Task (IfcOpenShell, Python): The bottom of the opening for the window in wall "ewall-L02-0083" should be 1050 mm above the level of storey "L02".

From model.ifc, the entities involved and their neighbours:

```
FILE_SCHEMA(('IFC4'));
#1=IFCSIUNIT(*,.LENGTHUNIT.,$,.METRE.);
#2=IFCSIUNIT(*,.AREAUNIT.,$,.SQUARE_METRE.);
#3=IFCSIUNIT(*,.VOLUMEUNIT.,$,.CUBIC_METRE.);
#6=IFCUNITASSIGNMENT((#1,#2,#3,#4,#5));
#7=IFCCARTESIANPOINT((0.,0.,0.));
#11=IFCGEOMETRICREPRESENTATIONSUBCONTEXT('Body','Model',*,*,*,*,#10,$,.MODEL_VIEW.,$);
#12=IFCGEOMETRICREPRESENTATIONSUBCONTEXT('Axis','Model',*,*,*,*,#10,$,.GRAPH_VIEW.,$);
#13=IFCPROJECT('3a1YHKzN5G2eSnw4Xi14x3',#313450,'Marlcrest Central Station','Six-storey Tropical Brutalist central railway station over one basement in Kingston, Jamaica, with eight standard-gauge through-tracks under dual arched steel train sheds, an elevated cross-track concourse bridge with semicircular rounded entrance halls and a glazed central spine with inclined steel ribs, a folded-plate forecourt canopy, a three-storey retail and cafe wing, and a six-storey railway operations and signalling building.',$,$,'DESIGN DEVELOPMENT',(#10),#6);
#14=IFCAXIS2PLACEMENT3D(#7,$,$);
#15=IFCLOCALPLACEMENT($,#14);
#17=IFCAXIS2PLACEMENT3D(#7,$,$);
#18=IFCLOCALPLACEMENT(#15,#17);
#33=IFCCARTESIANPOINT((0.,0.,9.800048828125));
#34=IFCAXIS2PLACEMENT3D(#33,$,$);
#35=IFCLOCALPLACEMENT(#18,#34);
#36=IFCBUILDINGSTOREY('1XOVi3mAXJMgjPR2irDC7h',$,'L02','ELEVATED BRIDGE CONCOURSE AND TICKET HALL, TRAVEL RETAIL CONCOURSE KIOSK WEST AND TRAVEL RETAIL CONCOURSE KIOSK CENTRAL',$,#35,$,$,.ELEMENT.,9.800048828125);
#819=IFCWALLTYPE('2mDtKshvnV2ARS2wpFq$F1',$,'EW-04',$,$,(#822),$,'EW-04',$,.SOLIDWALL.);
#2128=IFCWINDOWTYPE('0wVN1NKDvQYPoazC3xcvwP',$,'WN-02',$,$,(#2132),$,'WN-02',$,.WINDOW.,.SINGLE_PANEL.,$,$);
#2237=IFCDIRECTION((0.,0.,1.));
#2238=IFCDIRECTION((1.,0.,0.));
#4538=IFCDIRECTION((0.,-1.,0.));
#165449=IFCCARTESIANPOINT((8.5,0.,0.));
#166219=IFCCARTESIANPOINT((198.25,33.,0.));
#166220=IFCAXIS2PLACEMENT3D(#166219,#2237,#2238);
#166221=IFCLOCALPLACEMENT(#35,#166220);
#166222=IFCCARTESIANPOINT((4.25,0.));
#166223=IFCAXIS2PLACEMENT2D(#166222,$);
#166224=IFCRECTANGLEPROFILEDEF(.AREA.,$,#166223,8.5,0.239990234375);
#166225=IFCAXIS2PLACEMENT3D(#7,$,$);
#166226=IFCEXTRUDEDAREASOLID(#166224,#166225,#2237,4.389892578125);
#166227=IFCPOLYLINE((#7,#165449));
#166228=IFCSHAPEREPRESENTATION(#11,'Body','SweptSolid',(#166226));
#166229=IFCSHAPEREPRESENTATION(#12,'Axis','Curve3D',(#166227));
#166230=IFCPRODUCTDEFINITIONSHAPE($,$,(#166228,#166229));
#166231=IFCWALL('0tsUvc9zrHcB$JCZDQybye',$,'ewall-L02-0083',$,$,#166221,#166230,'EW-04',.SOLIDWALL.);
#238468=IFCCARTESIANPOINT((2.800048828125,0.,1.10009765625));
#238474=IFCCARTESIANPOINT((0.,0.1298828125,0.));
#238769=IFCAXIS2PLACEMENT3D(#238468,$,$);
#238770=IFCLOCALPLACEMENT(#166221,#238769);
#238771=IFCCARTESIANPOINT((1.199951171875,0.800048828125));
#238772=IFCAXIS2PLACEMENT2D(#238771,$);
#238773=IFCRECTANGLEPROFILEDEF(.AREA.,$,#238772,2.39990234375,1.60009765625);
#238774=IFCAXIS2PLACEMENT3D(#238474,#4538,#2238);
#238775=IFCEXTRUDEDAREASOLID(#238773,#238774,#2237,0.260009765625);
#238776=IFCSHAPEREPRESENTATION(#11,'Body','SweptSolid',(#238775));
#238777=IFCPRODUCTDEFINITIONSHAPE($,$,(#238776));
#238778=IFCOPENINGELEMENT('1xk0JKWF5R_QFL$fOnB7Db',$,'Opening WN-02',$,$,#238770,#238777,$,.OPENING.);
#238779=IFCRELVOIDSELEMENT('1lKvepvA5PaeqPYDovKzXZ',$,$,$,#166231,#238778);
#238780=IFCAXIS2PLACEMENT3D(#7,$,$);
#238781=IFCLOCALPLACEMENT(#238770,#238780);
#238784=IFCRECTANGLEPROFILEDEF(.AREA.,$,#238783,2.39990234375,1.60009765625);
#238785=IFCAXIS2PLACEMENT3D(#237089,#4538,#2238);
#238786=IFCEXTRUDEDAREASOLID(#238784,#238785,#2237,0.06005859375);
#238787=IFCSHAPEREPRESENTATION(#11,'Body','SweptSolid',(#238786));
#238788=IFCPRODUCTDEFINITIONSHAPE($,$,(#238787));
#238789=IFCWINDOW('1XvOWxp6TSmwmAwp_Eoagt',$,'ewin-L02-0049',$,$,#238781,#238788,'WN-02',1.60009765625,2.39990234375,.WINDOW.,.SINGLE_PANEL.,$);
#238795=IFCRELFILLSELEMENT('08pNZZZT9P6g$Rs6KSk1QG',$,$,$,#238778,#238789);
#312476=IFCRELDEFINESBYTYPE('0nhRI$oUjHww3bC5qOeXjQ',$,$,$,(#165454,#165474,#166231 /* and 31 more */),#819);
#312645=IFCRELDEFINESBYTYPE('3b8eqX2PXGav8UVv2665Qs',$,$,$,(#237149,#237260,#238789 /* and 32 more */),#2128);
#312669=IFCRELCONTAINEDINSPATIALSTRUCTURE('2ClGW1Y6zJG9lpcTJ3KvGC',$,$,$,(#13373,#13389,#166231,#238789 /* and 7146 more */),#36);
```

```python
import numpy as np
import ifcopenshell
import ifcopenshell.api.geometry
import ifcopenshell.geom
import ifcopenshell.util.element
import ifcopenshell.util.placement
import ifcopenshell.util.shape
import ifcopenshell.util.unit

model = ifcopenshell.open("model.ifc")
unit_scale = ifcopenshell.util.unit.calculate_unit_scale(model)

window = model.by_guid("1XvOWxp6TSmwmAwp_Eoagt")
opening = window.FillsVoids[0].RelatingOpeningElement
storey = ifcopenshell.util.element.get_container(window, ifc_class="IfcBuildingStorey")
level = ifcopenshell.util.placement.get_local_placement(storey.ObjectPlacement)[2, 3]

# The opening's origin need not be at the sill, so measure its lowest point.
shape = ifcopenshell.geom.create_shape(ifcopenshell.geom.settings(), opening)
bottom = ifcopenshell.util.shape.get_shape_bottom_elevation(shape, shape.geometry) / unit_scale
dz = level + 1.05 / unit_scale - bottom

shift = np.array([0.0, 0.0, dz])
# The window is placed relative to its opening, so it follows when the opening moves.
matrix = ifcopenshell.util.placement.get_local_placement(opening.ObjectPlacement)
matrix[:3, 3] += shift
ifcopenshell.api.geometry.edit_object_placement(
    model, product=opening, matrix=matrix, is_si=False, should_transform_children=True
)

print(f"moved by {dz * unit_scale:+.3f} m")

model.write("model_edited.ifc")
```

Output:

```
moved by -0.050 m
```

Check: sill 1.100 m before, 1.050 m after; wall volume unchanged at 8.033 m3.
